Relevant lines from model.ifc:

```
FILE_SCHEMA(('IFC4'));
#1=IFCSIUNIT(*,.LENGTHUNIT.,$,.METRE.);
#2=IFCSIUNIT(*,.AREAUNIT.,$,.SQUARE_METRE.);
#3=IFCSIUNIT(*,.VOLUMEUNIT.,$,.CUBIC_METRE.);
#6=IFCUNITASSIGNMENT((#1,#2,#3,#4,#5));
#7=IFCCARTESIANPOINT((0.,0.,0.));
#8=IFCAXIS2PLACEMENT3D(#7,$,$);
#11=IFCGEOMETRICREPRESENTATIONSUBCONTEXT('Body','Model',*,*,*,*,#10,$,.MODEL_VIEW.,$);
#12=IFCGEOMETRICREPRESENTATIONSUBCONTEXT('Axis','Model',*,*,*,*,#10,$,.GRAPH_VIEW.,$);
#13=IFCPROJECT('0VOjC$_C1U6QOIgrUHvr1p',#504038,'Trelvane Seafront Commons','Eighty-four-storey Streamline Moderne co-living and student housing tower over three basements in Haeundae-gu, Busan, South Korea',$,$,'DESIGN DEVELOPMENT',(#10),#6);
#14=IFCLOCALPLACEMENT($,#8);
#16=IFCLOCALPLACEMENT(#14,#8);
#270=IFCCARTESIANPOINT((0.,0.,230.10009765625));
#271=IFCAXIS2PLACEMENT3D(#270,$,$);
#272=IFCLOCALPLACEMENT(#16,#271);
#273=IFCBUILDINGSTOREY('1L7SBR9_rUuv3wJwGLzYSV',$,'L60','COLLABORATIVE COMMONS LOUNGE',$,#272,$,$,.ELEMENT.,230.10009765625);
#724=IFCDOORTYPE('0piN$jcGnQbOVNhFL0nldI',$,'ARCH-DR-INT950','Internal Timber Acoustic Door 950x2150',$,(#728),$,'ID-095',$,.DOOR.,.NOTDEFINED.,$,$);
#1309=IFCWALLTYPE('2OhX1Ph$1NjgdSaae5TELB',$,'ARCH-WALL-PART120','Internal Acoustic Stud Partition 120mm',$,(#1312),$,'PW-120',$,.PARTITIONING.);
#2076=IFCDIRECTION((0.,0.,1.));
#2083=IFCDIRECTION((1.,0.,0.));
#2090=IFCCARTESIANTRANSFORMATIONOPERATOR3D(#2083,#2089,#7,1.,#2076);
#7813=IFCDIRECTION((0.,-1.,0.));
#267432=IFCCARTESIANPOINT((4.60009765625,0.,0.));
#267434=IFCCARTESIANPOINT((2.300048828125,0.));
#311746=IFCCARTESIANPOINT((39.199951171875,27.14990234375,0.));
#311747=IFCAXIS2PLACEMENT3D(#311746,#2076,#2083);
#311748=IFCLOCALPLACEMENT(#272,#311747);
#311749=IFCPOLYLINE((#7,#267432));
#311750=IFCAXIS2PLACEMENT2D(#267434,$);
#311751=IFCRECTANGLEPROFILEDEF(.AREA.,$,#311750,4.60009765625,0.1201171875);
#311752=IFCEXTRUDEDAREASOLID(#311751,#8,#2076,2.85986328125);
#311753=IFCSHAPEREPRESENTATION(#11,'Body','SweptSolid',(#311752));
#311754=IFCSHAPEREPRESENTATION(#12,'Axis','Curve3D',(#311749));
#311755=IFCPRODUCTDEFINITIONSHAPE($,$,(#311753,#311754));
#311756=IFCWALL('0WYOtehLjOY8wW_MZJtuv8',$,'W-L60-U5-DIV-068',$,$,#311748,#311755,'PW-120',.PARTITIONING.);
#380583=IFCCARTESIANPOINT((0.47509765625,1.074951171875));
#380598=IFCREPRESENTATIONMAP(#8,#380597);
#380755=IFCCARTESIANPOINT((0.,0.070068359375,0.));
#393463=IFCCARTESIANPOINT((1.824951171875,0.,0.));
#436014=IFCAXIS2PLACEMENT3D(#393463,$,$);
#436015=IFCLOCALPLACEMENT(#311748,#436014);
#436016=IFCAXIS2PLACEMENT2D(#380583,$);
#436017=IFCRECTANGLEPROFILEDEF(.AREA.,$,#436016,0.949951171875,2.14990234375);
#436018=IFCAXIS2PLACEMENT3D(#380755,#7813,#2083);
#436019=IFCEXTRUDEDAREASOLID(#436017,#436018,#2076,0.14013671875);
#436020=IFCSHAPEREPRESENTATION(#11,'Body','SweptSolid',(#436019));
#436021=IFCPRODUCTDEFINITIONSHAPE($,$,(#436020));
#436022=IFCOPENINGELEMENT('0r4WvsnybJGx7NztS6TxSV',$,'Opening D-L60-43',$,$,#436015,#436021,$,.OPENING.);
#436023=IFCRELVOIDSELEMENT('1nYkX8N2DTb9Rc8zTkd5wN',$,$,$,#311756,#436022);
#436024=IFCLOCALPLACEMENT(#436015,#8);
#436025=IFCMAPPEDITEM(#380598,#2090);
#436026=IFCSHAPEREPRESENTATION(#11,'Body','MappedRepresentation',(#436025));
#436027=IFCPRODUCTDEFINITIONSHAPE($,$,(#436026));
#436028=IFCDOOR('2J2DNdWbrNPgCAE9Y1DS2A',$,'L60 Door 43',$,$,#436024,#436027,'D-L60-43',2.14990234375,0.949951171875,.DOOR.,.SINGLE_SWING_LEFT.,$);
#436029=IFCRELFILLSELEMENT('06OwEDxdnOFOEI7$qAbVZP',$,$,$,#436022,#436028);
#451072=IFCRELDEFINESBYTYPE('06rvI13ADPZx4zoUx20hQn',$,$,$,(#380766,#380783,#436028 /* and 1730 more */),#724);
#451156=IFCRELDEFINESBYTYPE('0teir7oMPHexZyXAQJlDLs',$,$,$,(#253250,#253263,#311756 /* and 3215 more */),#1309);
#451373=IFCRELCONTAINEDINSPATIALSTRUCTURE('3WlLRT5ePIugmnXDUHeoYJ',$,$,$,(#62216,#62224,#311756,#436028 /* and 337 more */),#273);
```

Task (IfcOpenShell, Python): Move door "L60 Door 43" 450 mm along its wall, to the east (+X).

```python
import ifcopenshell
import ifcopenshell.api.geometry
import ifcopenshell.util.placement

model = ifcopenshell.open("model.ifc")

door = model.by_id(436028)
opening = door.FillsVoids[0].RelatingOpeningElement
wall = opening.VoidsElements[0].RelatingBuildingElement

wall_matrix = ifcopenshell.util.placement.get_local_placement(wall.ObjectPlacement)
shift = wall_matrix[:3, 0] * 0.45
before = ifcopenshell.util.placement.get_local_placement(door.ObjectPlacement)[:3, 3].copy()

# The door is placed relative to its opening, so it follows when the opening moves.
matrix = ifcopenshell.util.placement.get_local_placement(opening.ObjectPlacement)
matrix[:3, 3] += shift
ifcopenshell.api.geometry.edit_object_placement(
    model, product=opening, matrix=matrix, is_si=False, should_transform_children=True
)

after = ifcopenshell.util.placement.get_local_placement(door.ObjectPlacement)[:3, 3]
print("door moved by", (after - before).round(3) + 0.0)

model.write("model_v2.ifc")
```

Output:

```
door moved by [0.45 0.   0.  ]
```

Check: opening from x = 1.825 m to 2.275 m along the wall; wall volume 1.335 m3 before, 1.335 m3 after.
